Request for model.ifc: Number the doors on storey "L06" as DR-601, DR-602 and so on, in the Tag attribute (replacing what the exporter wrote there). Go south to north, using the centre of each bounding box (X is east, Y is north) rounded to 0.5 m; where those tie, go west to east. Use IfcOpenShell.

First a look at what the model holds.

```python
import ifcopenshell
import ifcopenshell.util.element
import ifcopenshell.util.placement

model = ifcopenshell.open("model.ifc")
print(model.schema)
storey = next(s for s in model.by_type("IfcBuildingStorey") if s.Name == "L06")
doors = [e for e in ifcopenshell.util.element.get_decomposition(storey) if e.is_a("IfcDoor")]
for e in sorted(doors, key=lambda e: e.id()):
    origin = ifcopenshell.util.placement.get_local_placement(e.ObjectPlacement)[:3, 3]
    print(e.id(), e.Tag, e.Name, origin.round(2) + 0.0, sep=" | ")
```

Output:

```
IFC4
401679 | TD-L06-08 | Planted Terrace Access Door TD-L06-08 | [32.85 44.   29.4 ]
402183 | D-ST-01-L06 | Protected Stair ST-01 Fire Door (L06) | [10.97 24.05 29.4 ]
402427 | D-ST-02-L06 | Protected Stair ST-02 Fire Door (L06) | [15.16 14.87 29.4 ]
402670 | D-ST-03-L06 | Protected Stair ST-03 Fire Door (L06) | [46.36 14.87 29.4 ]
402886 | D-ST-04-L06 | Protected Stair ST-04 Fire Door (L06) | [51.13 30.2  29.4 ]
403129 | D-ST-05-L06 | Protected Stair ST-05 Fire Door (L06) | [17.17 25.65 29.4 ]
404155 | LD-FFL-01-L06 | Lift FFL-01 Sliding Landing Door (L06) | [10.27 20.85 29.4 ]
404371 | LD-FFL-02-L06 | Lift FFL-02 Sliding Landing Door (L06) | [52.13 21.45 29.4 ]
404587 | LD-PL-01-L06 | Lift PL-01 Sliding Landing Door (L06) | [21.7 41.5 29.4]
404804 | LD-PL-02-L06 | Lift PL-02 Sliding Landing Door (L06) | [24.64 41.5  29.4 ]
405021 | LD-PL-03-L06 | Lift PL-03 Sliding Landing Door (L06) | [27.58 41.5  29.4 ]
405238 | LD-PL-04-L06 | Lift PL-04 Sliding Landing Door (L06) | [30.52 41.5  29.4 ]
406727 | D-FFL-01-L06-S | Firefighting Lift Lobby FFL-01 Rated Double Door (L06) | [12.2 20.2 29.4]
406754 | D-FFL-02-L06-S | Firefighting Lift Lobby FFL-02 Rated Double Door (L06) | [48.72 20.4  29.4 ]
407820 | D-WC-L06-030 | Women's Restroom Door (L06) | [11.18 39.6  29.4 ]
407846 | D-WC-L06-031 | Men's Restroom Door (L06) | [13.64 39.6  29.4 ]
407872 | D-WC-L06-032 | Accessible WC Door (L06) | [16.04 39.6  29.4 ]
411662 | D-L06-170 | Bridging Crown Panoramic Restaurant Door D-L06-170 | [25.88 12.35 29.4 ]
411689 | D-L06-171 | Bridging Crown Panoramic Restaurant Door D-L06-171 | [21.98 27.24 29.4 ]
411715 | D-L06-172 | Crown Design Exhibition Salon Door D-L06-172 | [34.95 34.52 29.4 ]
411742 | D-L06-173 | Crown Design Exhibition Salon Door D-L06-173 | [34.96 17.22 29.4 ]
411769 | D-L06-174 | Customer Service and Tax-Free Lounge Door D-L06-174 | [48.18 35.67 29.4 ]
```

```python
import ifcopenshell
import ifcopenshell.geom
import ifcopenshell.util.element
import ifcopenshell.util.shape

model = ifcopenshell.open("model.ifc")
settings = ifcopenshell.geom.settings()
settings.set("use-world-coords", True)


def centre(element):
    shape = ifcopenshell.geom.create_shape(settings, element)
    return ifcopenshell.util.shape.get_bbox_centroid(shape.geometry)


storey = next(s for s in model.by_type("IfcBuildingStorey") if s.Name == "L06")
doors = [e for e in ifcopenshell.util.element.get_decomposition(storey) if e.is_a("IfcDoor")]

# Insertion points can sit at a corner or the storey origin, so sort by the geometry (in metres).
centres = {e: centre(e) for e in doors}
doors.sort(key=lambda e: (round(centres[e][1] / 0.5), centres[e][0]))

for i, e in enumerate(doors, start=1):
    number = f"DR-6{i:02d}"
    e.Tag = number
    print(e.id(), number)

model.write("model-out.ifc")
```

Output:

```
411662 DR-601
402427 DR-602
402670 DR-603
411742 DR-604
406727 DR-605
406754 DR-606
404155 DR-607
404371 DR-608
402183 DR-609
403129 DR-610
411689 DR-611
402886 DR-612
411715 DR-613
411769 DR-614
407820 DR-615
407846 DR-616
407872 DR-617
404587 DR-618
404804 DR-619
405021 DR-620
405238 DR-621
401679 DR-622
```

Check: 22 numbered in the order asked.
